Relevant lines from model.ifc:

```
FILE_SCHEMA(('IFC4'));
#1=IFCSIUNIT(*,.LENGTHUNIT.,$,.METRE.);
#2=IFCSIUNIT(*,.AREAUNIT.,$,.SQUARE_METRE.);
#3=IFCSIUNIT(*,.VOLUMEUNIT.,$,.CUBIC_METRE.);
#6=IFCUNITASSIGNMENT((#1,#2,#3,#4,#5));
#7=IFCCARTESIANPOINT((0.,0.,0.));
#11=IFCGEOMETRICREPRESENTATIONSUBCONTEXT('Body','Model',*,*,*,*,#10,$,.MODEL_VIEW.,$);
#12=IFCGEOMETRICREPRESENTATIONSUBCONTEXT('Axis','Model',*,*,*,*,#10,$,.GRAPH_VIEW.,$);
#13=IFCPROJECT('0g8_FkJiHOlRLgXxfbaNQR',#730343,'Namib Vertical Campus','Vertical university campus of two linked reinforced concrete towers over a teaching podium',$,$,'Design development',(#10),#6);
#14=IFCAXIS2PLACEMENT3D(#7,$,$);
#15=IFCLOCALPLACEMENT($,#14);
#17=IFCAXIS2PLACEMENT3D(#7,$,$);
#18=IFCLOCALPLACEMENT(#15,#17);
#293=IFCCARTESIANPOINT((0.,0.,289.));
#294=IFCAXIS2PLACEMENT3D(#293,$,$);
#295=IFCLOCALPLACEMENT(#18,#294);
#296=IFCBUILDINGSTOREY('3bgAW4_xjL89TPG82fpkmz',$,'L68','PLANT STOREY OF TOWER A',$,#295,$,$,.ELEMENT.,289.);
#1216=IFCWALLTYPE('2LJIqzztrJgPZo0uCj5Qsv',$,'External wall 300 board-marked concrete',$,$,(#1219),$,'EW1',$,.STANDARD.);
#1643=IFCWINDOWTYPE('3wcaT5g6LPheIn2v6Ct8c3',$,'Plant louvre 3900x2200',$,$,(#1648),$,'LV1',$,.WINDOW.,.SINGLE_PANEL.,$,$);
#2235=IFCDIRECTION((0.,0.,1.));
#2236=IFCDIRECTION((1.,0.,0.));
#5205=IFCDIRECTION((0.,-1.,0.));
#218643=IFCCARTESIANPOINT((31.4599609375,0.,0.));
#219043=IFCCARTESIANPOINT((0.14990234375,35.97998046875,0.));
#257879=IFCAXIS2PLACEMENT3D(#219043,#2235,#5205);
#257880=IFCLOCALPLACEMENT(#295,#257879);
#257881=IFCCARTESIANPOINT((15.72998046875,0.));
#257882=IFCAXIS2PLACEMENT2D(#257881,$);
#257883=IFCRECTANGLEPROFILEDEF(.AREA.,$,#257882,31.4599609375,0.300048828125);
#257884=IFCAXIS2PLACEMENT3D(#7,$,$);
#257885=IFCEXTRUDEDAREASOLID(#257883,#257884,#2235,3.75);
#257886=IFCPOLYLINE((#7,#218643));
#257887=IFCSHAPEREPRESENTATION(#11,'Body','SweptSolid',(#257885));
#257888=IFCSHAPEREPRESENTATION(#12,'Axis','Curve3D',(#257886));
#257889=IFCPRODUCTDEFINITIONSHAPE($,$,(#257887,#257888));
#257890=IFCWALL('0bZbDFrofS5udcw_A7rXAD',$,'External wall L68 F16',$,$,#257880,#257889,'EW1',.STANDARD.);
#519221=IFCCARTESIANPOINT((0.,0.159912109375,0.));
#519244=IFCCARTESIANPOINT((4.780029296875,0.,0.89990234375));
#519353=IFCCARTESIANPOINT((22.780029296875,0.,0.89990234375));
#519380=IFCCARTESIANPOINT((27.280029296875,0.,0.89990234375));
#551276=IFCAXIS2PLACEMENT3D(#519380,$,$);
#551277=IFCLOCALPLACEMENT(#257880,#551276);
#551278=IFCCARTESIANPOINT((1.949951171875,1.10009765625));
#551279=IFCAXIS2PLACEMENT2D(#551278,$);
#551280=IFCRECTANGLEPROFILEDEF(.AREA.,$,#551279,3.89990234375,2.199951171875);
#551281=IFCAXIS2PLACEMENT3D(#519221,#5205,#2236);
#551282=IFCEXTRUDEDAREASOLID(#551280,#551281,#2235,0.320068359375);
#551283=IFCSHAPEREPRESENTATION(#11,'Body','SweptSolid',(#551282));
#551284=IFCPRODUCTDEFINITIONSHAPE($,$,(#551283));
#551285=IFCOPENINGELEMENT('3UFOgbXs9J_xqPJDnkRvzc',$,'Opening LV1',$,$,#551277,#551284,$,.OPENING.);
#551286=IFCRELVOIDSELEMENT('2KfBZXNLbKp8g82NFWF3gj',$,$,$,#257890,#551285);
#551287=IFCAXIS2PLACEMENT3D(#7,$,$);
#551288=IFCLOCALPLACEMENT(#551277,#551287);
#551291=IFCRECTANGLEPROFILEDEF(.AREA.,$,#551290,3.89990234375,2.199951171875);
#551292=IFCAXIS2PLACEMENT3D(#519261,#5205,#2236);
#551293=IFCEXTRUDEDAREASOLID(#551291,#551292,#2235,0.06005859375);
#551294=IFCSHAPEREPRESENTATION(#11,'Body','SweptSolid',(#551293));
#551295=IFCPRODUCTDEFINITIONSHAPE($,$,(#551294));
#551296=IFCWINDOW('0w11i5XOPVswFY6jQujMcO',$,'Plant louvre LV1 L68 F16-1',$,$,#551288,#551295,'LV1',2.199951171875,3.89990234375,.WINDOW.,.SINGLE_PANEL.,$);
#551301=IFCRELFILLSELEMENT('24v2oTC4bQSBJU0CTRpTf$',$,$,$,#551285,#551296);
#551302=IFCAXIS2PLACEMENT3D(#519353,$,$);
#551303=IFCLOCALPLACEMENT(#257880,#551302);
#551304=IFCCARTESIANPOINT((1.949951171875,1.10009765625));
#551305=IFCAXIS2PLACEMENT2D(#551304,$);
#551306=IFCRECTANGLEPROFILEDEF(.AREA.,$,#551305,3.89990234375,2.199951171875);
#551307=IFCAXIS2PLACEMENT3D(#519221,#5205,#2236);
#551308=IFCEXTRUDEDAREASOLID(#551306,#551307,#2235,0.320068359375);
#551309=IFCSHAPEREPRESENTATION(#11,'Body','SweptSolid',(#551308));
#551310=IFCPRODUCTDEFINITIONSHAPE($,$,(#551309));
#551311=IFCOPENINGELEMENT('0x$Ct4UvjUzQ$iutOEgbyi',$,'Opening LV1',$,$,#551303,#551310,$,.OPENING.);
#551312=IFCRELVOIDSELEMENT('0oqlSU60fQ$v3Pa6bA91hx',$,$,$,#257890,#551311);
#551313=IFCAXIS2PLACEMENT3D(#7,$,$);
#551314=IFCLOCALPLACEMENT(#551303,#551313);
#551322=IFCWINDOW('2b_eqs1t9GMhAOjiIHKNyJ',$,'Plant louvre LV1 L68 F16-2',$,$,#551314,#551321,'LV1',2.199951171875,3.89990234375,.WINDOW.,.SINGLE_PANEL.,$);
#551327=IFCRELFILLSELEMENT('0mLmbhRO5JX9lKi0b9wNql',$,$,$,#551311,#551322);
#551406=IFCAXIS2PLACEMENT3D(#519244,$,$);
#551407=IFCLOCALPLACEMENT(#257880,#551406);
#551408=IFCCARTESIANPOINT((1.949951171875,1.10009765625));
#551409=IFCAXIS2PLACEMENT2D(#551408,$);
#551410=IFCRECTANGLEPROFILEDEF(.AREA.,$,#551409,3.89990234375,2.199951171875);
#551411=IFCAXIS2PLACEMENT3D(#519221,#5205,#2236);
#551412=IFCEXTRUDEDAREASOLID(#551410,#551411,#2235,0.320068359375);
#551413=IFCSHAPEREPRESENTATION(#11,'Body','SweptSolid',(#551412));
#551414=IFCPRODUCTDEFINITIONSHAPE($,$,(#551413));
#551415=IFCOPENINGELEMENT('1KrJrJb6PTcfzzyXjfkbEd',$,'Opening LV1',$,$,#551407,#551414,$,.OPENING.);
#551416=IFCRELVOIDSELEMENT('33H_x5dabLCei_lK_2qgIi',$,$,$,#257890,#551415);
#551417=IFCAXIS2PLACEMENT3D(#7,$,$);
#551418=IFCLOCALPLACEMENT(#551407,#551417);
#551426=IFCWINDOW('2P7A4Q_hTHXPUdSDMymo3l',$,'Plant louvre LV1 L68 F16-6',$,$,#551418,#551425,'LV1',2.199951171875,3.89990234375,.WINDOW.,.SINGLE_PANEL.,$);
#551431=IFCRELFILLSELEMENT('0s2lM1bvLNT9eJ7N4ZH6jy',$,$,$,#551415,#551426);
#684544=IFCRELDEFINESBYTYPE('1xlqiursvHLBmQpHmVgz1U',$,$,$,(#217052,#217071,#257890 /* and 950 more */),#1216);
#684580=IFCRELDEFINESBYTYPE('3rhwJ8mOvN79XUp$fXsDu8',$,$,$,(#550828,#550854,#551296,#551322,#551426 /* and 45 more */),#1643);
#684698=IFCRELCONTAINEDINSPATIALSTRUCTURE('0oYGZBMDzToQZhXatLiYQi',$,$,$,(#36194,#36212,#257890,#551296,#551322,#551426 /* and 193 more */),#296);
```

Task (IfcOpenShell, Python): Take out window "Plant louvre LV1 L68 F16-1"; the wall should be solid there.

```python
import ifcopenshell
import ifcopenshell.api.feature
import ifcopenshell.api.root
import ifcopenshell.geom
import ifcopenshell.util.shape

model = ifcopenshell.open("model.ifc")
settings = ifcopenshell.geom.settings()


def volume(element):
    """Net volume in cubic metres, openings subtracted."""
    shape = ifcopenshell.geom.create_shape(settings, element)
    return ifcopenshell.util.shape.get_volume(shape.geometry)


window = model.by_guid("0w11i5XOPVswFY6jQujMcO")
opening = window.FillsVoids[0].RelatingOpeningElement
wall = opening.VoidsElements[0].RelatingBuildingElement
before = volume(wall)

ifcopenshell.api.root.remove_product(model, product=window)
ifcopenshell.api.feature.remove_feature(model, feature=opening)

after = volume(wall)

print(f"wall volume {before:.3f} -> {after:.3f} m3")

model.write("model_updated.ifc")
```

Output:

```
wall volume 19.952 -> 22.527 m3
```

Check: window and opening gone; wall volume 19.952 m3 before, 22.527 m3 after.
